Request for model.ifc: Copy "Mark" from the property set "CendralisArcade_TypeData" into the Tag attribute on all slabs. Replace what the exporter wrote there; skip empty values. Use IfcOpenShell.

First a look at what the model holds.

```python
import ifcopenshell
import ifcopenshell.util.element

model = ifcopenshell.open("model.ifc")
print(model.schema)
slabs = model.by_type("IfcSlab")
print(len(slabs), "slabs")
for e in slabs[:8]:
    source = ifcopenshell.util.element.get_pset(e, "CendralisArcade_TypeData", "Mark")
    target = e.Tag
    print(e.id(), repr(source), repr(target), sep=" | ")
```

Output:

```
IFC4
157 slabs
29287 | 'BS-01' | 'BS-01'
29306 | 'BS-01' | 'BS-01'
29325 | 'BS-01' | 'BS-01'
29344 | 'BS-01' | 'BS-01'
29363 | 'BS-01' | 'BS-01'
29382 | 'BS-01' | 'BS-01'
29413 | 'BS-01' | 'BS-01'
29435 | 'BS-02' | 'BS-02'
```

```python
import ifcopenshell
import ifcopenshell.util.element

model = ifcopenshell.open("model.ifc")

count = 0
for e in model.by_type("IfcSlab"):
    value = ifcopenshell.util.element.get_pset(e, "CendralisArcade_TypeData", "Mark")
    current = e.Tag
    if not value or not value.strip() or current == value:
        continue
    e.Tag = value
    count += 1

print(count, "slabs updated")

model.write("model_updated.ifc")
```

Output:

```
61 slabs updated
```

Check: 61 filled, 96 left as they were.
